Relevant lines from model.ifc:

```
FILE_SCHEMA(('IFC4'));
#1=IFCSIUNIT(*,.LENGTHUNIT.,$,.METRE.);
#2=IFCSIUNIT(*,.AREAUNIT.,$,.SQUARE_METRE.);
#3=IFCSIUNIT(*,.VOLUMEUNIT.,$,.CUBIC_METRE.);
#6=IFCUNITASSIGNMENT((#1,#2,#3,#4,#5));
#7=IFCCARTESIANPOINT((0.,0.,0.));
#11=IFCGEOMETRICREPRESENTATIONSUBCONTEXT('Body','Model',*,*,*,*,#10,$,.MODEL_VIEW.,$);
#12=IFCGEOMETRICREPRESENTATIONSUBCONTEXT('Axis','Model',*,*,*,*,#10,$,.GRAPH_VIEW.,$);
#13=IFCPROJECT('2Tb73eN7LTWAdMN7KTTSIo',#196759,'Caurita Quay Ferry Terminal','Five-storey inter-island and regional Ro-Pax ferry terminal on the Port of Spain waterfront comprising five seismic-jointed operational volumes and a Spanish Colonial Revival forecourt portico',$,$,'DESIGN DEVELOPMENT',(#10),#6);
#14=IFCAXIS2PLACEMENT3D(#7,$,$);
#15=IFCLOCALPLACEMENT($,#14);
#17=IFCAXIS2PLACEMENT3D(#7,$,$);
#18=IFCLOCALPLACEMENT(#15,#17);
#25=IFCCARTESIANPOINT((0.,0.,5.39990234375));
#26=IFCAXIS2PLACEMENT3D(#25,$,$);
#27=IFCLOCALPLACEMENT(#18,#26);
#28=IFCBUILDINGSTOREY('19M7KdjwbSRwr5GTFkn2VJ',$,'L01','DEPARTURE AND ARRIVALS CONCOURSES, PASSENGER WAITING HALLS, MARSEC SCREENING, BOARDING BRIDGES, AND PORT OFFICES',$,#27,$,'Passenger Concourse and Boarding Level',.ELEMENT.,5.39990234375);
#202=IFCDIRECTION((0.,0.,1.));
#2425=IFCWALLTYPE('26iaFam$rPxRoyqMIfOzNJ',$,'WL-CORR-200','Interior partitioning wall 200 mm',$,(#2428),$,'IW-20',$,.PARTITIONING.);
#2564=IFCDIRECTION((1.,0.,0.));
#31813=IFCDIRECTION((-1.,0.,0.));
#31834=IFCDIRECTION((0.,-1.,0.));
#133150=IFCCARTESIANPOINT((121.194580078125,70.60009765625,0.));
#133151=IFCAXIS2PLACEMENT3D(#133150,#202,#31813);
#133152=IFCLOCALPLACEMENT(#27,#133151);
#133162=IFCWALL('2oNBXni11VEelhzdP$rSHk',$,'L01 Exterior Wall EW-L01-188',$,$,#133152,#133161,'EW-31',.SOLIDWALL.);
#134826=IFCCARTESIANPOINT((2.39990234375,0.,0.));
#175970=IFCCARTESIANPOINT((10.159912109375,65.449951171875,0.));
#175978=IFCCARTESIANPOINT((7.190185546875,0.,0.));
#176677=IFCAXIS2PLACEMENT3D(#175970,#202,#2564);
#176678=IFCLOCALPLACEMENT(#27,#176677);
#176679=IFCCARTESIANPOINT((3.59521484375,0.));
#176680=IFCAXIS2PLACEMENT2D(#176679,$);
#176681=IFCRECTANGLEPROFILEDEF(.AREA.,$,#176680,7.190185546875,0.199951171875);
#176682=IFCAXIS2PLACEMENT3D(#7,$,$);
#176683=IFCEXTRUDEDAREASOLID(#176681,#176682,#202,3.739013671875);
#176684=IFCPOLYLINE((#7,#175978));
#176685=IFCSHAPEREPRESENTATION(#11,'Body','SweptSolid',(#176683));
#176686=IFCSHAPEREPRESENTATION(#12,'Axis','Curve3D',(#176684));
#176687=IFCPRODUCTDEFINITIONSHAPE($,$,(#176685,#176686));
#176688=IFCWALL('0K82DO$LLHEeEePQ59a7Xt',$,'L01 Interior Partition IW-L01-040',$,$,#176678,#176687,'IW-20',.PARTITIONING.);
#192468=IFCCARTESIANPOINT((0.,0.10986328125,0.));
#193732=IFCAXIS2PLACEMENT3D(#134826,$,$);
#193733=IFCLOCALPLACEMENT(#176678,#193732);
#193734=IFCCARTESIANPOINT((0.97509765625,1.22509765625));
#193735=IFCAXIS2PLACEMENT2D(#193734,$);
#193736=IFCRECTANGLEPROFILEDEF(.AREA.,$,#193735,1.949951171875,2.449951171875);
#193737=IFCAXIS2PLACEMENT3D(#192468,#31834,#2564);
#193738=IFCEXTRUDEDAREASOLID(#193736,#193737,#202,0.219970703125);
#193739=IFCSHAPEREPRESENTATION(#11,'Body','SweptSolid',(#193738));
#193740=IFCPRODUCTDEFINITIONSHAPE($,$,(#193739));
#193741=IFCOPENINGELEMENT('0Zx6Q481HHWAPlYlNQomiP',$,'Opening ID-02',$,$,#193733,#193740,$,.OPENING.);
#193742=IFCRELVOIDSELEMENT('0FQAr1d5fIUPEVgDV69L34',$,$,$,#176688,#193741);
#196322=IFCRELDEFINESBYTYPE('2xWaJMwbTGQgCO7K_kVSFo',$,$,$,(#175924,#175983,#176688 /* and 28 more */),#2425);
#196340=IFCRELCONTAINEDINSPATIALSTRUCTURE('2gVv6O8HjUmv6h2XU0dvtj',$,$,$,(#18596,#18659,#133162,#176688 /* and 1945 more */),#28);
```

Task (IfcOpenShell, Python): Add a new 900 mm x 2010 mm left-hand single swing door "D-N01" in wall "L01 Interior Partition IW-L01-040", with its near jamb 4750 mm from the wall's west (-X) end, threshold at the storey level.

```python
import numpy as np
import ifcopenshell
import ifcopenshell.api.feature
import ifcopenshell.api.geometry
import ifcopenshell.api.root
import ifcopenshell.api.spatial
import ifcopenshell.geom
import ifcopenshell.util.element
import ifcopenshell.util.placement
import ifcopenshell.util.representation
import ifcopenshell.util.shape
import ifcopenshell.util.unit

model = ifcopenshell.open("model.ifc")
unit_scale = ifcopenshell.util.unit.calculate_unit_scale(model)
settings = ifcopenshell.geom.settings()


def volume(element):
    """Net volume in cubic metres, openings subtracted."""
    shape = ifcopenshell.geom.create_shape(settings, element)
    return ifcopenshell.util.shape.get_volume(shape.geometry)


wall = model.by_guid("0K82DO$LLHEeEePQ59a7Xt")
storey = ifcopenshell.util.element.get_container(wall, ifc_class="IfcBuildingStorey")
context = ifcopenshell.util.representation.get_context(model, "Model", "Body", "MODEL_VIEW")
before = volume(wall)

width, height, from_end, sill = 0.9, 2.01, 4.75, 0.0  # metres

# The wall runs along its own X axis, and the end named is its -X end.
wall_shape = ifcopenshell.geom.create_shape(settings, wall)
x, y, z = ifcopenshell.util.shape.get_vertices(wall_shape.geometry).T
start = x.min() + from_end
face, thickness = float(y.min()), float(y.max() - y.min())
wall_matrix = ifcopenshell.util.placement.get_local_placement(wall.ObjectPlacement)
level = ifcopenshell.util.placement.get_local_placement(storey.ObjectPlacement)[2, 3]


def in_wall(x, y):
    """Placement at x, y metres in the wall's axes, at sill height."""
    matrix = wall_matrix.copy()
    matrix[:, 3] = wall_matrix @ np.array([x / unit_scale, y / unit_scale, 0.0, 1.0])
    matrix[2, 3] = level + sill / unit_scale
    return matrix


# Opening: a box that overshoots both wall faces by 50 mm.
opening = ifcopenshell.api.root.create_entity(model, ifc_class="IfcOpeningElement", predefined_type="OPENING")
box = ifcopenshell.api.geometry.add_wall_representation(
    model, context=context, length=width, height=height, thickness=thickness + 0.1
)
ifcopenshell.api.geometry.assign_representation(model, product=opening, representation=box)
ifcopenshell.api.geometry.edit_object_placement(model, product=opening, matrix=in_wall(start, face - 0.05), is_si=False)
ifcopenshell.api.feature.add_feature(model, feature=opening, element=wall)

door = ifcopenshell.api.root.create_entity(model, ifc_class="IfcDoor", name="D-N01", predefined_type="DOOR")
door.OverallWidth, door.OverallHeight = width / unit_scale, height / unit_scale
door.OperationType = "SINGLE_SWING_LEFT"
body = ifcopenshell.api.geometry.add_door_representation(
    model,
    context=context,
    overall_width=door.OverallWidth,
    overall_height=door.OverallHeight,
    operation_type="SINGLE_SWING_LEFT",
    lining_properties={"LiningDepth": thickness / unit_scale, "ThresholdDepth": thickness / unit_scale},
)
ifcopenshell.api.geometry.assign_representation(model, product=door, representation=body)
ifcopenshell.api.spatial.assign_container(model, products=[door], relating_structure=storey)
ifcopenshell.api.feature.add_filling(model, opening=opening, element=door)

# The lining spans the wall, so the door starts at the wall face.
ifcopenshell.api.geometry.edit_object_placement(model, product=door, matrix=in_wall(start, face), is_si=False)

after = volume(wall)

print(f"wall volume {before:.3f} -> {after:.3f} m3")

model.write("model_v2.ifc")
```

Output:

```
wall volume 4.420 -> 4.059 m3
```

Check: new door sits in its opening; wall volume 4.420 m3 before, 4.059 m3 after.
